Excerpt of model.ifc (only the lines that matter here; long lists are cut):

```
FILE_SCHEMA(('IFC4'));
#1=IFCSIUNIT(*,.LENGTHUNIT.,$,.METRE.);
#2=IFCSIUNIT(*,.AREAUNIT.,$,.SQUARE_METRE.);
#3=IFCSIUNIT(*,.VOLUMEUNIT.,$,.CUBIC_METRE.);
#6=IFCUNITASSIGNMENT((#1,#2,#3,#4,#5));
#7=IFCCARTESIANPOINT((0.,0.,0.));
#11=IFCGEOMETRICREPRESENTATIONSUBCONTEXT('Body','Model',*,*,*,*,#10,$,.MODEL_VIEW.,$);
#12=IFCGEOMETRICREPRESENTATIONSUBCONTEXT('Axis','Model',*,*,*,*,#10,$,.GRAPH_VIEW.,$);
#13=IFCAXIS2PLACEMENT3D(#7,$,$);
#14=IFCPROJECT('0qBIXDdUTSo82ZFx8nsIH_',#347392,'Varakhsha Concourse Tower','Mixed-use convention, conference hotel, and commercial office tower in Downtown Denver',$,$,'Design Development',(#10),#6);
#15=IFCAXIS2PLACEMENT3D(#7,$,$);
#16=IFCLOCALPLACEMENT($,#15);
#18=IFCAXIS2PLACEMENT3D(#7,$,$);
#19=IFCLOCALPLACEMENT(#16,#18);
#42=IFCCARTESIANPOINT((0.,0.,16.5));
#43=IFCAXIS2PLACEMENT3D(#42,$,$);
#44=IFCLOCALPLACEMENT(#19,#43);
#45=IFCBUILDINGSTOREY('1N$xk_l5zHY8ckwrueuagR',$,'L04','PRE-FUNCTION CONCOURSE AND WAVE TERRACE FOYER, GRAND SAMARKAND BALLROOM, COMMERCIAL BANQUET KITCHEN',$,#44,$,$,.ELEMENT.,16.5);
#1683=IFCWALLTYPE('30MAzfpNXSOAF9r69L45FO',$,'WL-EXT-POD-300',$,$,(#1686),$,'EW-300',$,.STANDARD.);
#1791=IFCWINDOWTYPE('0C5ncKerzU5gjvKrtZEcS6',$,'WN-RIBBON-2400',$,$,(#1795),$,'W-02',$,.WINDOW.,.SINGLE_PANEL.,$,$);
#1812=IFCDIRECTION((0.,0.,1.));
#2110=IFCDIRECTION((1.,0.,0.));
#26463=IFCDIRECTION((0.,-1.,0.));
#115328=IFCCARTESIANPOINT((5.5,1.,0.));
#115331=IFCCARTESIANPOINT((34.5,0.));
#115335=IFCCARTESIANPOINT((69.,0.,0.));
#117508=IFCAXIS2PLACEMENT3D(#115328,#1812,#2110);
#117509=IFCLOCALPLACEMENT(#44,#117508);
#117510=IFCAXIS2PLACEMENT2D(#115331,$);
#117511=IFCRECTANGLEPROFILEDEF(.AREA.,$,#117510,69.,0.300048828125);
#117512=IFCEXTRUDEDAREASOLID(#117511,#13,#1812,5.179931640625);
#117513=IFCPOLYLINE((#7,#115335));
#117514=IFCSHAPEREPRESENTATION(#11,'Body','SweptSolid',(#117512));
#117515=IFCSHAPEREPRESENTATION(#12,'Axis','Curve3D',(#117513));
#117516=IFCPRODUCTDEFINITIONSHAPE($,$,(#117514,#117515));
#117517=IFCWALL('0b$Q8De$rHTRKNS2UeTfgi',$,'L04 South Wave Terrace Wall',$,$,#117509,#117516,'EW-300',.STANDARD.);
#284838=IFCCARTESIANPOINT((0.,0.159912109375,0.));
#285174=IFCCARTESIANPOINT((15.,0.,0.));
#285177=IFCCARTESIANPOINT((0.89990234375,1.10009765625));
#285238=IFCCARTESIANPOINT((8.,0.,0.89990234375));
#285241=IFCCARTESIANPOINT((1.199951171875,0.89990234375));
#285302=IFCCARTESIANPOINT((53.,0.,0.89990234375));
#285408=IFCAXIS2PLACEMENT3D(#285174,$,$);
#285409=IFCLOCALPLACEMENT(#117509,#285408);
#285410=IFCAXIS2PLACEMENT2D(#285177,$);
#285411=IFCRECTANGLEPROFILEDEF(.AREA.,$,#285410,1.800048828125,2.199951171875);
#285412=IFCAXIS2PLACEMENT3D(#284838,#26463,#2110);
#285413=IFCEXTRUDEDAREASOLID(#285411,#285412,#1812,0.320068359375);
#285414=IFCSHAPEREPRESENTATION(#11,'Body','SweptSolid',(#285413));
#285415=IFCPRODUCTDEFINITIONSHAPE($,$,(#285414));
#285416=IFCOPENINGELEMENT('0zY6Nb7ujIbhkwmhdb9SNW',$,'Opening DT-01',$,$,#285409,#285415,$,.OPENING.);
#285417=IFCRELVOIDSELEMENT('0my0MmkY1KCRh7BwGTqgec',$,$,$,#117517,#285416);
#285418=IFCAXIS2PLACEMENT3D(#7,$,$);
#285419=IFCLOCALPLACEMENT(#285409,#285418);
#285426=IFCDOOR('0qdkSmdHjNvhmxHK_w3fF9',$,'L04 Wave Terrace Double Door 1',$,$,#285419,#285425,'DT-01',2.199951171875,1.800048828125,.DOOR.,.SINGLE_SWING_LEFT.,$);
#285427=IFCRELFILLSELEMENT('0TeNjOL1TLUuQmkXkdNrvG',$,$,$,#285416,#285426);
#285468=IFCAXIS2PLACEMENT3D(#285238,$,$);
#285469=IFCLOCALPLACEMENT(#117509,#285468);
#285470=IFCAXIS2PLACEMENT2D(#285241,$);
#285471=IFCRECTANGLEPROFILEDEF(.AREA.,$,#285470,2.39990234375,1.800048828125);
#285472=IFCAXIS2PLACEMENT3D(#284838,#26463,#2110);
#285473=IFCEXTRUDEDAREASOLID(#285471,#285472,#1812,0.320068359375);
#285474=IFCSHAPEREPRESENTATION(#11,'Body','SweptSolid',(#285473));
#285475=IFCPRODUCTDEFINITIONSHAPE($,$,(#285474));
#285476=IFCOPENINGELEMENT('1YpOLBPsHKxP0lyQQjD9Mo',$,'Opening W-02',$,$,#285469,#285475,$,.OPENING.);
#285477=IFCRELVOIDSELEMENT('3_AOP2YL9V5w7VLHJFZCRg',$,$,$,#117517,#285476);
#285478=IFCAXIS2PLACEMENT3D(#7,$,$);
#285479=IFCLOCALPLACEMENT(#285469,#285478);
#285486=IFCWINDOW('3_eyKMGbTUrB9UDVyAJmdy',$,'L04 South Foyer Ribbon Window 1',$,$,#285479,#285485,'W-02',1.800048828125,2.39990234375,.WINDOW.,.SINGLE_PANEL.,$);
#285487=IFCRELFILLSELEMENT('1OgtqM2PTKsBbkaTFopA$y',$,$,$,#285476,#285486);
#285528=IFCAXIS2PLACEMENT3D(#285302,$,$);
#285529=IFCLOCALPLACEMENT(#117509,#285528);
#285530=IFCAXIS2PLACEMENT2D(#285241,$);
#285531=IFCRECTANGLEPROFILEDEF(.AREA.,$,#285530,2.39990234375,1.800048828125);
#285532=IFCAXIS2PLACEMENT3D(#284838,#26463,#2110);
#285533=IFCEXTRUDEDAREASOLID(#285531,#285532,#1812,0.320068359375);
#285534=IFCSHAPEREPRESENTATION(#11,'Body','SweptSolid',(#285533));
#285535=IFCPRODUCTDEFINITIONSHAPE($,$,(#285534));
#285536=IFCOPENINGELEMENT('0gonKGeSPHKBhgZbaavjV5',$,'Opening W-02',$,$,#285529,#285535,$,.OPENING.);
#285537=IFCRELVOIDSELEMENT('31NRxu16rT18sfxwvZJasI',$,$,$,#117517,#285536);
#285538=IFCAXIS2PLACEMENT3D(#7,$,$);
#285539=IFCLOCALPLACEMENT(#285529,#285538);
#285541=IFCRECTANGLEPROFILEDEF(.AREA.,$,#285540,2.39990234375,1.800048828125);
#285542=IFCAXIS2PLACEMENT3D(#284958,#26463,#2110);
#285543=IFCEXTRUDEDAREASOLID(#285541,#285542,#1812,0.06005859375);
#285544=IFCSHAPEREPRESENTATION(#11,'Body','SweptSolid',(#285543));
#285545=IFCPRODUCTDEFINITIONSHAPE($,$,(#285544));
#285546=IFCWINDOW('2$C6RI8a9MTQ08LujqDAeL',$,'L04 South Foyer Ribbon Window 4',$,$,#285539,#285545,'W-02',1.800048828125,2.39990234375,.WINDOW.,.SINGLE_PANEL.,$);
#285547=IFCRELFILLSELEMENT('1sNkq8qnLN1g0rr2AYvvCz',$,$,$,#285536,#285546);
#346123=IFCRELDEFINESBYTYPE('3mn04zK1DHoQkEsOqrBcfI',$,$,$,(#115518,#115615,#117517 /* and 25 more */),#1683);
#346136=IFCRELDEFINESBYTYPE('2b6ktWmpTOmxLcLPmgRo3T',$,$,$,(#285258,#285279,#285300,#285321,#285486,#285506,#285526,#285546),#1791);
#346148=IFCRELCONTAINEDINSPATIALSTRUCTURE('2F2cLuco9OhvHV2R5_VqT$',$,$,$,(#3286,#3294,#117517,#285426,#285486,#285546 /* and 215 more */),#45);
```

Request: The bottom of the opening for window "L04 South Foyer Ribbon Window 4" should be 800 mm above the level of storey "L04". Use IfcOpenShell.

```python
import numpy as np
import ifcopenshell
import ifcopenshell.api.geometry
import ifcopenshell.geom
import ifcopenshell.util.element
import ifcopenshell.util.placement
import ifcopenshell.util.shape
import ifcopenshell.util.unit

model = ifcopenshell.open("model.ifc")
unit_scale = ifcopenshell.util.unit.calculate_unit_scale(model)

window = model.by_id(285546)
opening = window.FillsVoids[0].RelatingOpeningElement
storey = ifcopenshell.util.element.get_container(window, ifc_class="IfcBuildingStorey")
level = ifcopenshell.util.placement.get_local_placement(storey.ObjectPlacement)[2, 3]

# The opening's origin need not be at the sill, so measure its lowest point.
shape = ifcopenshell.geom.create_shape(ifcopenshell.geom.settings(), opening)
bottom = ifcopenshell.util.shape.get_shape_bottom_elevation(shape, shape.geometry) / unit_scale
dz = level + 0.8 - bottom

shift = np.array([0.0, 0.0, dz])
# The window is placed relative to its opening, so it follows when the opening moves.
matrix = ifcopenshell.util.placement.get_local_placement(opening.ObjectPlacement)
matrix[:3, 3] += shift
ifcopenshell.api.geometry.edit_object_placement(
    model, product=opening, matrix=matrix, is_si=False, should_transform_children=True
)

print(f"moved by {dz * unit_scale:+.3f} m")

model.write("model-out.ifc")
```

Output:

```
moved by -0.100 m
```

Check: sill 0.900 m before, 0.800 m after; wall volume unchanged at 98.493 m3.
